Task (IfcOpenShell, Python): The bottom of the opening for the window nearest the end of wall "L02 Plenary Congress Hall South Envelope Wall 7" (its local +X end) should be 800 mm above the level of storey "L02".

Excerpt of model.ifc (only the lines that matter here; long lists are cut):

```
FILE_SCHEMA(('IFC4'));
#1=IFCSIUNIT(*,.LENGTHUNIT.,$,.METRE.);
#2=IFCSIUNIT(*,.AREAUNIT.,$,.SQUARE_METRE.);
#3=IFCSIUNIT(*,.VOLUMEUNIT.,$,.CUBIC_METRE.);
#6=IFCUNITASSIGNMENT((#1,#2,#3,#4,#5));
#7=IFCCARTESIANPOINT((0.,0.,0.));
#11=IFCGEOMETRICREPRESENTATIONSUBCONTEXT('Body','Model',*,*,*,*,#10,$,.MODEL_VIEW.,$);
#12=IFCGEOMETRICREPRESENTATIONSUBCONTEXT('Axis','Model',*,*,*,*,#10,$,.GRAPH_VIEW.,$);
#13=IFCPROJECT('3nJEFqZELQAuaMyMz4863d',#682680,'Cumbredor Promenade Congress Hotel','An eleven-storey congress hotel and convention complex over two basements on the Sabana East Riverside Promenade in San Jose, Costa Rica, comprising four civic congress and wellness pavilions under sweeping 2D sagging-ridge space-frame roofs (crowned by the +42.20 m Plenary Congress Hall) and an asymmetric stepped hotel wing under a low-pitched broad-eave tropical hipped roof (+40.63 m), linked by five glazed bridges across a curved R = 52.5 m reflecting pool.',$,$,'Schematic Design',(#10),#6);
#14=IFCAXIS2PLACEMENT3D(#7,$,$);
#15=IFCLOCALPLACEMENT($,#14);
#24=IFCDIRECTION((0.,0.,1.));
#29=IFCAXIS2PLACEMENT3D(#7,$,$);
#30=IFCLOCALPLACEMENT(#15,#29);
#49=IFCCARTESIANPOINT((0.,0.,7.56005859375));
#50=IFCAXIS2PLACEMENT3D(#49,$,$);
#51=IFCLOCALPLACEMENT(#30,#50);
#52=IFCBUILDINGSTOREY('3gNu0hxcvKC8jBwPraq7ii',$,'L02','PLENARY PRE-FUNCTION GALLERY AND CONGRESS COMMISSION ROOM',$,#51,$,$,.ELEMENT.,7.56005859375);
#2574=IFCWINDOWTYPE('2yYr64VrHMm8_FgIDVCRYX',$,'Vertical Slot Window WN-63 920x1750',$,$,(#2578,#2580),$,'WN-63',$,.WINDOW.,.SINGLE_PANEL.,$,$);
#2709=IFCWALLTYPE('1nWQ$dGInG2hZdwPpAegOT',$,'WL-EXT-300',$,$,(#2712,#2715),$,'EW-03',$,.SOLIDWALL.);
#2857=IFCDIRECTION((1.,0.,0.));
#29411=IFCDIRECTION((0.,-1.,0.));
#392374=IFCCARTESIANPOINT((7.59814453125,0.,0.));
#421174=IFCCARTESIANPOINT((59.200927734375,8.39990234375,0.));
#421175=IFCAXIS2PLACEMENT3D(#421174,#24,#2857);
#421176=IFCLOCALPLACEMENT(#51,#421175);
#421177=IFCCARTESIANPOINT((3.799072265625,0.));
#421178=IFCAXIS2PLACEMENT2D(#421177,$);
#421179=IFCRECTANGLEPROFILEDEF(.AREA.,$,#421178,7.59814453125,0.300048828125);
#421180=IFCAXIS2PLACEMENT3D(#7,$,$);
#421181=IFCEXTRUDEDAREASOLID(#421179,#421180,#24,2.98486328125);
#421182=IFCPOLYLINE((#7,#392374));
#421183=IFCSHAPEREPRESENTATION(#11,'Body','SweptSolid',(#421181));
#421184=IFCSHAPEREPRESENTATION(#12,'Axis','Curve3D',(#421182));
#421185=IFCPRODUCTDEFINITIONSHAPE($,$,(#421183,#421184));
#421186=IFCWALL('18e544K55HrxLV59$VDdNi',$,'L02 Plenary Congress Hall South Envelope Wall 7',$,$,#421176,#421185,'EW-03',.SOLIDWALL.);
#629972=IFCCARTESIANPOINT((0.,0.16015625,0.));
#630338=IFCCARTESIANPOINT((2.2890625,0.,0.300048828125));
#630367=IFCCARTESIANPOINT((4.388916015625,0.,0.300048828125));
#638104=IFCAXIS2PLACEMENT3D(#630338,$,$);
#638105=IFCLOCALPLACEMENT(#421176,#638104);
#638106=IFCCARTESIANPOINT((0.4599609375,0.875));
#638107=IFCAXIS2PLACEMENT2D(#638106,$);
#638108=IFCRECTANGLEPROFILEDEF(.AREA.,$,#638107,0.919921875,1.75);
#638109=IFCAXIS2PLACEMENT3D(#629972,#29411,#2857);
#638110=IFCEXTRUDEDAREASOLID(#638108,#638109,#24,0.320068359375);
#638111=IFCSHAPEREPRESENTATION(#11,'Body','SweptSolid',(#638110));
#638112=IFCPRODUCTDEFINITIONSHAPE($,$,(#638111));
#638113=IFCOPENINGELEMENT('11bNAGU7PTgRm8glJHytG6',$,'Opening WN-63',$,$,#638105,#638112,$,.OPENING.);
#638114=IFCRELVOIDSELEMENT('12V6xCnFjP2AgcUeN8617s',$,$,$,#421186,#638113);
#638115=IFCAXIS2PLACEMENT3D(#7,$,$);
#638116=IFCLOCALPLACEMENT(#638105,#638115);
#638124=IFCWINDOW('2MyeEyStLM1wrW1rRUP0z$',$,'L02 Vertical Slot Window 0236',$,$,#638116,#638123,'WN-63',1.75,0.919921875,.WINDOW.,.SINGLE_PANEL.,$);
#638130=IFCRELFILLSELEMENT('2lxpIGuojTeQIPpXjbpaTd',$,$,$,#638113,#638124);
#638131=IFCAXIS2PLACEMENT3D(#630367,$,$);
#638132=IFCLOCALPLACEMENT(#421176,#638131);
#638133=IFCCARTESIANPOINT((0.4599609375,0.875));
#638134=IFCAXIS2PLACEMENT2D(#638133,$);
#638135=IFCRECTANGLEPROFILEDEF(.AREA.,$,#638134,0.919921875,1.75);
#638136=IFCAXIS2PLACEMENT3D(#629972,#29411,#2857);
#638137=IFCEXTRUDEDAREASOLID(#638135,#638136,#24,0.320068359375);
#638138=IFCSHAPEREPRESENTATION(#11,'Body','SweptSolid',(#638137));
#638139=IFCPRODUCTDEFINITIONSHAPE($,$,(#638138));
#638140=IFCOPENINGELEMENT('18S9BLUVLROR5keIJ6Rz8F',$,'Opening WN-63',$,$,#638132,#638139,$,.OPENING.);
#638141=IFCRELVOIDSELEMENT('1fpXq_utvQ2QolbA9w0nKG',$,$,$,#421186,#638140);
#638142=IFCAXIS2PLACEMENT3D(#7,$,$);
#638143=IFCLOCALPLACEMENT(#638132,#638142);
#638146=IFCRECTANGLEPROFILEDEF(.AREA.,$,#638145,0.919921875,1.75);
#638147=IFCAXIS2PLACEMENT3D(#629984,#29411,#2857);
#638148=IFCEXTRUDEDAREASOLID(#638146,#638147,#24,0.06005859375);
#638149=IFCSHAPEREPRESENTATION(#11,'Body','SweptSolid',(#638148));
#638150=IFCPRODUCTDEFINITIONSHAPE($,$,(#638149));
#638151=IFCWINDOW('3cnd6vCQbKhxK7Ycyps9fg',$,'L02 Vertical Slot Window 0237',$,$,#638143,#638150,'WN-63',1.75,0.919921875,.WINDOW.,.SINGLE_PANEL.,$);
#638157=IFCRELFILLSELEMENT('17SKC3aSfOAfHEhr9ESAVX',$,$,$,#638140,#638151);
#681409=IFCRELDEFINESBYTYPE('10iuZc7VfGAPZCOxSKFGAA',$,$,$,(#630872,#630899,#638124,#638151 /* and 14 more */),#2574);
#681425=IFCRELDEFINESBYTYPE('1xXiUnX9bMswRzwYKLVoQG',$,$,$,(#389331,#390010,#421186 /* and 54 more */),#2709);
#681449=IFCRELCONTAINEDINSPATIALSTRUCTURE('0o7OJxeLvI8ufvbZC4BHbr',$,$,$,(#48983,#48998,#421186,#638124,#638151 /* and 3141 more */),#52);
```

```python
import numpy as np
import ifcopenshell
import ifcopenshell.api.geometry
import ifcopenshell.geom
import ifcopenshell.util.element
import ifcopenshell.util.placement
import ifcopenshell.util.shape
import ifcopenshell.util.unit

model = ifcopenshell.open("model.ifc")
unit_scale = ifcopenshell.util.unit.calculate_unit_scale(model)

window = model.by_guid("3cnd6vCQbKhxK7Ycyps9fg")
opening = window.FillsVoids[0].RelatingOpeningElement
storey = ifcopenshell.util.element.get_container(window, ifc_class="IfcBuildingStorey")
level = ifcopenshell.util.placement.get_local_placement(storey.ObjectPlacement)[2, 3]

# The opening's origin need not be at the sill, so measure its lowest point.
shape = ifcopenshell.geom.create_shape(ifcopenshell.geom.settings(), opening)
bottom = ifcopenshell.util.shape.get_shape_bottom_elevation(shape, shape.geometry) / unit_scale
dz = level + 0.8 / unit_scale - bottom

shift = np.array([0.0, 0.0, dz])
# The window is placed relative to its opening, so it follows when the opening moves.
matrix = ifcopenshell.util.placement.get_local_placement(opening.ObjectPlacement)
matrix[:3, 3] += shift
ifcopenshell.api.geometry.edit_object_placement(
    model, product=opening, matrix=matrix, is_si=False, should_transform_children=True
)

print(f"moved by {dz * unit_scale:+.3f} m")

model.write("model-out.ifc")
```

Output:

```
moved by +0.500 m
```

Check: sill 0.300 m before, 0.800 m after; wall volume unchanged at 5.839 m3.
